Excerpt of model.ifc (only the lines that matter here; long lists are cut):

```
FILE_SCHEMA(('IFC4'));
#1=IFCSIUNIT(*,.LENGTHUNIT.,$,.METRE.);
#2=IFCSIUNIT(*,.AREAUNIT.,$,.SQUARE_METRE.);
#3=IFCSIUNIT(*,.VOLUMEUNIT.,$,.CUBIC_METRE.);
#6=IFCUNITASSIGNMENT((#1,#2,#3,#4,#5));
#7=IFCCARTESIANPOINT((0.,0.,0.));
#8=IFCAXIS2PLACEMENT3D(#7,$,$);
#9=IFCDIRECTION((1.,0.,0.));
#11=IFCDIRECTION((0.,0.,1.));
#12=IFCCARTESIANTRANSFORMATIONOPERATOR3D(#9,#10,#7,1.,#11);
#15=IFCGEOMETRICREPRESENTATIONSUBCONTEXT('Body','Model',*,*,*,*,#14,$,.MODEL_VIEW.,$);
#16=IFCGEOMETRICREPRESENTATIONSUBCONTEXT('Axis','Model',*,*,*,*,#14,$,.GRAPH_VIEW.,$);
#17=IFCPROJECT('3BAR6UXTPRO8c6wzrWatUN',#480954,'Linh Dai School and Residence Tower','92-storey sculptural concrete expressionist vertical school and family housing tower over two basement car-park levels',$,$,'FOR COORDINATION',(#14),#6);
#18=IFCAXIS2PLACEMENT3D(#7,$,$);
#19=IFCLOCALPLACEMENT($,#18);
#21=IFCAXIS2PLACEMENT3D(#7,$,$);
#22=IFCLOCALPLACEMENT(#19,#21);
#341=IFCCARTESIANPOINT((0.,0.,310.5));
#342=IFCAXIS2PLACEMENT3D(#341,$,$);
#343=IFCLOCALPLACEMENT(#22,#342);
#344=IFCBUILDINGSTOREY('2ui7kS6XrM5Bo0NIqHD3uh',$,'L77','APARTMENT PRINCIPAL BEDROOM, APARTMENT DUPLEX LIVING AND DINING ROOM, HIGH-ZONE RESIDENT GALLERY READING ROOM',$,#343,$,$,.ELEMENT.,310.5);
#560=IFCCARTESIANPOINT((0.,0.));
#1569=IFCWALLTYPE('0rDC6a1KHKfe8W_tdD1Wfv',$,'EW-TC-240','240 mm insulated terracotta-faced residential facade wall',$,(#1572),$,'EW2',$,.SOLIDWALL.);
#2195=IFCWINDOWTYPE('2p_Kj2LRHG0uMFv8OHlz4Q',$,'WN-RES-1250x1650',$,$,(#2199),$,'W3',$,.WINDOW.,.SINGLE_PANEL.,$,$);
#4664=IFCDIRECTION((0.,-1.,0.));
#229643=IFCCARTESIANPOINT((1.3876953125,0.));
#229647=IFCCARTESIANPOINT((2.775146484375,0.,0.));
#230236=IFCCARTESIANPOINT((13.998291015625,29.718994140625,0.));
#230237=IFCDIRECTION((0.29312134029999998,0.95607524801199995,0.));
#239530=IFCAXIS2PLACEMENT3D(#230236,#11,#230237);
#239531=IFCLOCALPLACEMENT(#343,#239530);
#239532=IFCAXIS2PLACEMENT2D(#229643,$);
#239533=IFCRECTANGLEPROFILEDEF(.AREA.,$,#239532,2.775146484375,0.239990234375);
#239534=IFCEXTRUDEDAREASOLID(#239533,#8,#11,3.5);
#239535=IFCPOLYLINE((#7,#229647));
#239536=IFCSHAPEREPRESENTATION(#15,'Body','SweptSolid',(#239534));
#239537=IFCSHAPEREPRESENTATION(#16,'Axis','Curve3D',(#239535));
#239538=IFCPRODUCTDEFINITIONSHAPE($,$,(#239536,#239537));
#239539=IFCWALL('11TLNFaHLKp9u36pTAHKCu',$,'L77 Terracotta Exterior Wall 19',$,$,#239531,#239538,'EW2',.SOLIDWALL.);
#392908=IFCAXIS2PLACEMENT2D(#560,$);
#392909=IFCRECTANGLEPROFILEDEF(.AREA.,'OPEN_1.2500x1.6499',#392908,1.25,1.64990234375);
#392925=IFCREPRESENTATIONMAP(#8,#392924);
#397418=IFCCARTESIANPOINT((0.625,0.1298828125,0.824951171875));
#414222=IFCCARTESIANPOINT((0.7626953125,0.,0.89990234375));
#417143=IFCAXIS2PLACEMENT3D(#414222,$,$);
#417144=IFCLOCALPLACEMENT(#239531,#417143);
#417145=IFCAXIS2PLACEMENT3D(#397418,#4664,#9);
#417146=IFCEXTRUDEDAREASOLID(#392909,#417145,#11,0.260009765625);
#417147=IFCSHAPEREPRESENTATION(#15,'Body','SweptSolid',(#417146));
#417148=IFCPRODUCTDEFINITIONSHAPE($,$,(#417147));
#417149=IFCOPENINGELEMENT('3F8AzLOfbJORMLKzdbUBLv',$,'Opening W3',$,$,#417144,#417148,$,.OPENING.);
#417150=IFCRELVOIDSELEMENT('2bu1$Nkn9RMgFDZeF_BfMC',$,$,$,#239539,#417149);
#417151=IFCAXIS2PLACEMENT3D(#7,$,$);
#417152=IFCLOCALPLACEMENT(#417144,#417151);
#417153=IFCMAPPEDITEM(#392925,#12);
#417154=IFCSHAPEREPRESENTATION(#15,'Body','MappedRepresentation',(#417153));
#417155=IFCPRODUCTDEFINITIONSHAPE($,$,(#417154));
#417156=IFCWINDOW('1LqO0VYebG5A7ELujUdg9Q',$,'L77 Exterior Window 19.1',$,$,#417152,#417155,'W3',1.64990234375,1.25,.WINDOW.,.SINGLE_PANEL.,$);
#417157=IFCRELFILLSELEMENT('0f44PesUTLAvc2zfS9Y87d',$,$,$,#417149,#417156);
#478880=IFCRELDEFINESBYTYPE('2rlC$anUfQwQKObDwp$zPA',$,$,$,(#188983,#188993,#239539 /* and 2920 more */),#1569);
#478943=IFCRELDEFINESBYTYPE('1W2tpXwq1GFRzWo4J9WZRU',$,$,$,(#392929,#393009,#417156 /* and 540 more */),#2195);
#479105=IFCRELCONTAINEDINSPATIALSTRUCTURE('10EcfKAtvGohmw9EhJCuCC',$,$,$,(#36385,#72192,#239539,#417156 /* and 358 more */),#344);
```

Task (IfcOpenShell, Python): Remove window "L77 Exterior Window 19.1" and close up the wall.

```python
import ifcopenshell
import ifcopenshell.api.feature
import ifcopenshell.api.root
import ifcopenshell.geom
import ifcopenshell.util.shape

model = ifcopenshell.open("model.ifc")
settings = ifcopenshell.geom.settings()


def volume(element):
    """Net volume in cubic metres, openings subtracted."""
    shape = ifcopenshell.geom.create_shape(settings, element)
    return ifcopenshell.util.shape.get_volume(shape.geometry)


window = model.by_guid("1LqO0VYebG5A7ELujUdg9Q")
opening = window.FillsVoids[0].RelatingOpeningElement
wall = opening.VoidsElements[0].RelatingBuildingElement
before = volume(wall)

ifcopenshell.api.root.remove_product(model, product=window)
ifcopenshell.api.feature.remove_feature(model, feature=opening)

after = volume(wall)

print(f"wall volume {before:.3f} -> {after:.3f} m3")

model.write("model_edited.ifc")
```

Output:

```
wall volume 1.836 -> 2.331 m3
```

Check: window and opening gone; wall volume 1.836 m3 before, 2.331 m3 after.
